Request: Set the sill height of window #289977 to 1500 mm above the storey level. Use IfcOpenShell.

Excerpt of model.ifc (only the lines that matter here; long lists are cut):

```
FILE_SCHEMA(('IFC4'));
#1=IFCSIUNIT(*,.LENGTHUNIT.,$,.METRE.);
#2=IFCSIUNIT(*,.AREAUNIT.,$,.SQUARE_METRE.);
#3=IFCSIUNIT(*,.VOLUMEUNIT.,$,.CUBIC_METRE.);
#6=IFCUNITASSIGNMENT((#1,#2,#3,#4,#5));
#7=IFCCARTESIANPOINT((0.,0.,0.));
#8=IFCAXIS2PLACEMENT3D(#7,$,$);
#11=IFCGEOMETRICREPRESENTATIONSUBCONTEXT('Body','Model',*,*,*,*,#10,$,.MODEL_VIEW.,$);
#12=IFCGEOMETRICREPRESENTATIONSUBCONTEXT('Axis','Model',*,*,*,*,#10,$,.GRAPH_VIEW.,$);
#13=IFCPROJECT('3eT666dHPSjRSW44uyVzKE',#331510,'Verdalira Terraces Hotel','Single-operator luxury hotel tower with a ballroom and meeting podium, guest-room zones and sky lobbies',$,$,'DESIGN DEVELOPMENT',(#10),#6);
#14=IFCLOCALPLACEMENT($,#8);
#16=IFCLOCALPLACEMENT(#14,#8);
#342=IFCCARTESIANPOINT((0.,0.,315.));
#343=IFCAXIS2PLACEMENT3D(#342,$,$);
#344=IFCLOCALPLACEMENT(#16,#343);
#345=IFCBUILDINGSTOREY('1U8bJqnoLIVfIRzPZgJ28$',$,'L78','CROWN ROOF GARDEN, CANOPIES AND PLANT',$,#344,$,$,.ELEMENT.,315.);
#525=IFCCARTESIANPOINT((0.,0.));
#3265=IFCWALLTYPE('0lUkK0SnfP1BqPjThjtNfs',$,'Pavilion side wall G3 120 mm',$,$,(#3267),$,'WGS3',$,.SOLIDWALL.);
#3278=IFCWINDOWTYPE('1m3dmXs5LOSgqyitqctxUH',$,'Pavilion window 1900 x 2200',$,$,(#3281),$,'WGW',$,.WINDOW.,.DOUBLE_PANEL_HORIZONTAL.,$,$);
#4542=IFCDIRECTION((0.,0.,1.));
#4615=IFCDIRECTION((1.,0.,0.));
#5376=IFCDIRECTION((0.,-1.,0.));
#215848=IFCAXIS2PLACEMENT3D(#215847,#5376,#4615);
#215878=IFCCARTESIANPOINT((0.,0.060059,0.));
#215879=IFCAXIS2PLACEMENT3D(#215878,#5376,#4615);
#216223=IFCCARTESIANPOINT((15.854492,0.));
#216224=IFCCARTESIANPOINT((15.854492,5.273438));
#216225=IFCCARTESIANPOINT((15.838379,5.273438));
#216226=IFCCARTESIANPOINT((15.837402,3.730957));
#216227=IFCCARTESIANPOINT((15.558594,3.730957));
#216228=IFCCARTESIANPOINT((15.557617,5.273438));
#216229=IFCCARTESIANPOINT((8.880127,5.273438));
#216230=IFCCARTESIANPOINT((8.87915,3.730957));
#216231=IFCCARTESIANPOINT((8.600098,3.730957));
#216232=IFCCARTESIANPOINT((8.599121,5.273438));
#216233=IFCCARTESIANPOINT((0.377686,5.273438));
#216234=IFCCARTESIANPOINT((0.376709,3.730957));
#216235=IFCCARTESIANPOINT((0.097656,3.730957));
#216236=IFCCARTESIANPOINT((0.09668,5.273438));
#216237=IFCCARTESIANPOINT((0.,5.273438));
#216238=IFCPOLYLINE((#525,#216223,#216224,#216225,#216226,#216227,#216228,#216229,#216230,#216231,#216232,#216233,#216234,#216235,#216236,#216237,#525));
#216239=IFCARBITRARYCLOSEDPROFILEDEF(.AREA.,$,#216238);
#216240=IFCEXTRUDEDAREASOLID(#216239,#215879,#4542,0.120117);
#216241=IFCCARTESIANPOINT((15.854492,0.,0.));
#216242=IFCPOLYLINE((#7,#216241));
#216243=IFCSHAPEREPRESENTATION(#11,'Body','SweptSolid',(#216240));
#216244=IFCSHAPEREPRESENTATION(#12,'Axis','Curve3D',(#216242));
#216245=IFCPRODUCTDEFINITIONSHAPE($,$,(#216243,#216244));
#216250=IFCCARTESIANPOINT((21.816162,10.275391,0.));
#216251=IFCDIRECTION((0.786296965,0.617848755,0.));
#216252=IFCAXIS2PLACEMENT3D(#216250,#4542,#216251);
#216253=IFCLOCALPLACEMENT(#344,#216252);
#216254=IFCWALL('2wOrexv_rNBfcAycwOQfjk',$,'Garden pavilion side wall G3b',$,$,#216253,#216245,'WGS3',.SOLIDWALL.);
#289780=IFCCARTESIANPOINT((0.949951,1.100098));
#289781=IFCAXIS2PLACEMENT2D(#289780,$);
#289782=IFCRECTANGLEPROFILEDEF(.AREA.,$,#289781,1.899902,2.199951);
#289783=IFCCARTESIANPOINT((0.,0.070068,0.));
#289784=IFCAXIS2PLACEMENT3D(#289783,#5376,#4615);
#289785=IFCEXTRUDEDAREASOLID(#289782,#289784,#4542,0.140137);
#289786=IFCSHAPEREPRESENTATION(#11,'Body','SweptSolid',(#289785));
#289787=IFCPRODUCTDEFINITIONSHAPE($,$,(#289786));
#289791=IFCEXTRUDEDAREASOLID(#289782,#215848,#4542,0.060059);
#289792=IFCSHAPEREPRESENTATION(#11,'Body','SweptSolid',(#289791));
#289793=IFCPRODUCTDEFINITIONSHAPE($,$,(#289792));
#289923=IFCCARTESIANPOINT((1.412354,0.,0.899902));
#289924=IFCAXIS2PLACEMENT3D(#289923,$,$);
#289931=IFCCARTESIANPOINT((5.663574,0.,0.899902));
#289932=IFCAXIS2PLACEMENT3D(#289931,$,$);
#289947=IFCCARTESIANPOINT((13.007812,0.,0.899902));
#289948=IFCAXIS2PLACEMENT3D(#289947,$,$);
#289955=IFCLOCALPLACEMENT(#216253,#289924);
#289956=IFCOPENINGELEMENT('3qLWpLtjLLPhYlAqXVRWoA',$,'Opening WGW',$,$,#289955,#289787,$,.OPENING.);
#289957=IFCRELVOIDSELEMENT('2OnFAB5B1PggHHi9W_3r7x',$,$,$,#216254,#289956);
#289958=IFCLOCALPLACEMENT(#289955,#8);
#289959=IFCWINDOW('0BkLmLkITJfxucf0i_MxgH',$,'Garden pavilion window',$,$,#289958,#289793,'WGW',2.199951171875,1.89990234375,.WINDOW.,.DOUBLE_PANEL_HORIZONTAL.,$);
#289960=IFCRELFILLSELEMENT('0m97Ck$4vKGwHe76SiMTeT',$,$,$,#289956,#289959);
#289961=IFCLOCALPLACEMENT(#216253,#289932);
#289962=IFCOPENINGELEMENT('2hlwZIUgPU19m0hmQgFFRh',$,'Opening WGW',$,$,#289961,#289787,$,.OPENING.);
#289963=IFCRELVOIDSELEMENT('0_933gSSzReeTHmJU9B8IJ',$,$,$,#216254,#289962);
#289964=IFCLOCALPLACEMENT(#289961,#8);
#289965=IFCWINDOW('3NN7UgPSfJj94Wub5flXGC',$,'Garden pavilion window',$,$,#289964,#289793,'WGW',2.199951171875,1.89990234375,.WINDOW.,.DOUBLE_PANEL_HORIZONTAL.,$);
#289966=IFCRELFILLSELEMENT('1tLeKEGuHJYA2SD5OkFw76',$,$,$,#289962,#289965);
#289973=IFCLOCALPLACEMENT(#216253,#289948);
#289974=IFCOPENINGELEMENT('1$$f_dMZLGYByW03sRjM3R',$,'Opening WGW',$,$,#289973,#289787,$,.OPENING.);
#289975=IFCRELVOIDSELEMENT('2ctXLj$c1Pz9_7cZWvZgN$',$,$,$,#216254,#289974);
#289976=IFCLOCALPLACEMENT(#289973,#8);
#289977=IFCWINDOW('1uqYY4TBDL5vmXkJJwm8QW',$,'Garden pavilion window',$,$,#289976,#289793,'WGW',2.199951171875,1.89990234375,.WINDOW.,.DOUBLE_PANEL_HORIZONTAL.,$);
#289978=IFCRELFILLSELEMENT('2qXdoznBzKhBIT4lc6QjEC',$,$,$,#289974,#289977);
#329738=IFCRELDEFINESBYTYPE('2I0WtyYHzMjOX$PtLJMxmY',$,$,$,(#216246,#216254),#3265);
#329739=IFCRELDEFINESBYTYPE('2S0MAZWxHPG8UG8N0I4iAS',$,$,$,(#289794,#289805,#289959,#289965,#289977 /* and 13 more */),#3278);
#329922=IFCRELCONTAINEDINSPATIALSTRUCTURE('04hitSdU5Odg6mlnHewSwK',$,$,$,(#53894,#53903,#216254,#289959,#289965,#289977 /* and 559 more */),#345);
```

```python
import numpy as np
import ifcopenshell
import ifcopenshell.api.geometry
import ifcopenshell.geom
import ifcopenshell.util.element
import ifcopenshell.util.placement
import ifcopenshell.util.shape
import ifcopenshell.util.unit

model = ifcopenshell.open("model.ifc")
unit_scale = ifcopenshell.util.unit.calculate_unit_scale(model)

window = model.by_guid("1uqYY4TBDL5vmXkJJwm8QW")
opening = window.FillsVoids[0].RelatingOpeningElement
storey = ifcopenshell.util.element.get_container(window, ifc_class="IfcBuildingStorey")
level = ifcopenshell.util.placement.get_local_placement(storey.ObjectPlacement)[2, 3]

# The opening's origin need not be at the sill, so measure its lowest point.
shape = ifcopenshell.geom.create_shape(ifcopenshell.geom.settings(), opening)
bottom = ifcopenshell.util.shape.get_shape_bottom_elevation(shape, shape.geometry) / unit_scale
dz = level + 1.5 / unit_scale - bottom

shift = np.array([0.0, 0.0, dz])
# The window is placed relative to its opening, so it follows when the opening moves.
matrix = ifcopenshell.util.placement.get_local_placement(opening.ObjectPlacement)
matrix[:3, 3] += shift
ifcopenshell.api.geometry.edit_object_placement(
    model, product=opening, matrix=matrix, is_si=False, should_transform_children=True
)

print(f"moved by {dz * unit_scale:+.3f} m")

model.write("model_rev.ifc")
```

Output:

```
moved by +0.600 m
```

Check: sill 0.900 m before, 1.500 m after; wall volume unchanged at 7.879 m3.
